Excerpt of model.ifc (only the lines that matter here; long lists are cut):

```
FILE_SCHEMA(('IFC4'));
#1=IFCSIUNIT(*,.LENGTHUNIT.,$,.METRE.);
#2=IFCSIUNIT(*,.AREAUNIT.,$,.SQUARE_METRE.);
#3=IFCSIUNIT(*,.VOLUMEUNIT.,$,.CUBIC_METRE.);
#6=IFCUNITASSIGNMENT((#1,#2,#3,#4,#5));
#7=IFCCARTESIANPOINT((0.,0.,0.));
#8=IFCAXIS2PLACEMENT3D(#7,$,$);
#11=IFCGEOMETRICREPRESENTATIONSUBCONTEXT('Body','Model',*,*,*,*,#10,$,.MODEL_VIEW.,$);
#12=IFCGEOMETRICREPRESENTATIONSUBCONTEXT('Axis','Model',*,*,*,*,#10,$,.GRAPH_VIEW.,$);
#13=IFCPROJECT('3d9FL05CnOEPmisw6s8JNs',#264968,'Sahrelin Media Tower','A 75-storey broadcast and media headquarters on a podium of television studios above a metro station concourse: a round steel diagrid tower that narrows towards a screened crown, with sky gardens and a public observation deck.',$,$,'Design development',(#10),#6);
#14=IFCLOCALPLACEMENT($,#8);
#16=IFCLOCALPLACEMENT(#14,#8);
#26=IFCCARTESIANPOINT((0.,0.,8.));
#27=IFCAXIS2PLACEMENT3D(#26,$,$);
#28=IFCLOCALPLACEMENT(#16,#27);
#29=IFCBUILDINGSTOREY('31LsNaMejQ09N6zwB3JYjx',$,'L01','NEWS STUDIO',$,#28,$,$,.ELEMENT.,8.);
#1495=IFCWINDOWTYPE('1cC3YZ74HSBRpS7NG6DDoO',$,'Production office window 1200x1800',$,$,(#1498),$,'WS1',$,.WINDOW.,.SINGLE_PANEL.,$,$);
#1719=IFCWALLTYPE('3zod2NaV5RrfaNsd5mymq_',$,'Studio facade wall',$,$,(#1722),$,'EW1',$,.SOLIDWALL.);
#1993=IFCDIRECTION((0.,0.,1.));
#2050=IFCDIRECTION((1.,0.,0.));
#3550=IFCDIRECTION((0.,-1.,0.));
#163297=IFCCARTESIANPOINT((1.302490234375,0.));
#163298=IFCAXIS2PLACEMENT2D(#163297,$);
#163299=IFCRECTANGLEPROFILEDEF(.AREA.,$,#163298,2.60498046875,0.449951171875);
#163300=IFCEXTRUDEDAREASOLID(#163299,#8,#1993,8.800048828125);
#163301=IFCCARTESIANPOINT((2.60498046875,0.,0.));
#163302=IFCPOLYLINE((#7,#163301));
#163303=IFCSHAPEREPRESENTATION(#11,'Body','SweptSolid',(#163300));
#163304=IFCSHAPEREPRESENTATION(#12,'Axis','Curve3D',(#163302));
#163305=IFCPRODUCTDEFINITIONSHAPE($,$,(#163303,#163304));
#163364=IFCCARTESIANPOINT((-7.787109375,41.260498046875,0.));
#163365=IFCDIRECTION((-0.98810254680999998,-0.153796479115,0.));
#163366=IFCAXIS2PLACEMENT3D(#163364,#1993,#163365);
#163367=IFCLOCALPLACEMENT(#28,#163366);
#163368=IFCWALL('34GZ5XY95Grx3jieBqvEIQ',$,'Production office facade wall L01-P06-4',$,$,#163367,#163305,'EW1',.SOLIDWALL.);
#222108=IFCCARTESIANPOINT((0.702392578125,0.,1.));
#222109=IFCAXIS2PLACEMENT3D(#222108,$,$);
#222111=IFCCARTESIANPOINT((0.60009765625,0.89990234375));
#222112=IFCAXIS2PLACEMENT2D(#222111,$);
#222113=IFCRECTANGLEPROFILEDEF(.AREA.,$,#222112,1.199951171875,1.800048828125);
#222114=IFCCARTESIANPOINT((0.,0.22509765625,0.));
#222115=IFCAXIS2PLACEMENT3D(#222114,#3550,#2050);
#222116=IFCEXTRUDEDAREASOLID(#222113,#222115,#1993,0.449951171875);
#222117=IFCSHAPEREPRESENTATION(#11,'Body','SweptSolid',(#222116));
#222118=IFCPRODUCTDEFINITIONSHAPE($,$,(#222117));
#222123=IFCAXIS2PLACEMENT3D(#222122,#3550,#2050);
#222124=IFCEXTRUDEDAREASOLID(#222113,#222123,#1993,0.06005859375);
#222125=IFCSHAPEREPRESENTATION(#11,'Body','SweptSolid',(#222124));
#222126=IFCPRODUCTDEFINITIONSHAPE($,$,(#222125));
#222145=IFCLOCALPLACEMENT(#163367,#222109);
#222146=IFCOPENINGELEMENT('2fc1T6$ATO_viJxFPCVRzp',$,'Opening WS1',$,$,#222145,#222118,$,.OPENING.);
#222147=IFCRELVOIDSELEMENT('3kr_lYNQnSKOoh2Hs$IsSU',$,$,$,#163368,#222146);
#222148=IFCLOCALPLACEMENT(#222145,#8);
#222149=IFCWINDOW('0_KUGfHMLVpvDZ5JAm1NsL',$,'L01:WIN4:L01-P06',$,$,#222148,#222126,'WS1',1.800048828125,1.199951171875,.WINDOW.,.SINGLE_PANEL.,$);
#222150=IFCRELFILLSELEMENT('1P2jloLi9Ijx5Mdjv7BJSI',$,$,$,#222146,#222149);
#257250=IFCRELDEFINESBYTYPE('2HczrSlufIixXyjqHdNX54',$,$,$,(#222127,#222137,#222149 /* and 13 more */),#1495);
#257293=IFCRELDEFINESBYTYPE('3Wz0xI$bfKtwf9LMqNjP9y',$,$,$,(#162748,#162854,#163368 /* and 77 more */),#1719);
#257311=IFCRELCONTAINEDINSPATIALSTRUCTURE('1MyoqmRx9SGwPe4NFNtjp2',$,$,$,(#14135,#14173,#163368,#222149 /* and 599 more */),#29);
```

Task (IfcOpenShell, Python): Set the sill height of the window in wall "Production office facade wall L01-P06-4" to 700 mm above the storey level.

```python
import numpy as np
import ifcopenshell
import ifcopenshell.api.geometry
import ifcopenshell.geom
import ifcopenshell.util.element
import ifcopenshell.util.placement
import ifcopenshell.util.shape
import ifcopenshell.util.unit

model = ifcopenshell.open("model.ifc")
unit_scale = ifcopenshell.util.unit.calculate_unit_scale(model)

window = model.by_id(222149)
opening = window.FillsVoids[0].RelatingOpeningElement
storey = ifcopenshell.util.element.get_container(window, ifc_class="IfcBuildingStorey")
level = ifcopenshell.util.placement.get_local_placement(storey.ObjectPlacement)[2, 3]

# The opening's origin need not be at the sill, so measure its lowest point.
shape = ifcopenshell.geom.create_shape(ifcopenshell.geom.settings(), opening)
bottom = ifcopenshell.util.shape.get_shape_bottom_elevation(shape, shape.geometry) / unit_scale
dz = level + 0.7 / unit_scale - bottom

shift = np.array([0.0, 0.0, dz])
# The window is placed relative to its opening, so it follows when the opening moves.
matrix = ifcopenshell.util.placement.get_local_placement(opening.ObjectPlacement)
matrix[:3, 3] += shift
ifcopenshell.api.geometry.edit_object_placement(
    model, product=opening, matrix=matrix, is_si=False, should_transform_children=True
)

print(f"moved by {dz * unit_scale:+.3f} m")

model.write("model_edited.ifc")
```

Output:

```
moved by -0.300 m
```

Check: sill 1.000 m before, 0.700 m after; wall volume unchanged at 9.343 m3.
